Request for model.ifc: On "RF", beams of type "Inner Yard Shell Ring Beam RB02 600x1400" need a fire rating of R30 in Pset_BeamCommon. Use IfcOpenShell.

First a look at what the model holds.

```python
import ifcopenshell
import ifcopenshell.util.element

model = ifcopenshell.open("model.ifc")
print(model.schema)
storey = next(s for s in model.by_type("IfcBuildingStorey") if s.Name == "RF")
beams = [e for e in ifcopenshell.util.element.get_decomposition(storey) if e.is_a("IfcBeam")]
seen = {}
for e in beams:
    element_type = ifcopenshell.util.element.get_type(e)
    key = (element_type.Name if element_type != e and element_type else None, ifcopenshell.util.element.get_pset(e, "Pset_BeamCommon", "FireRating"))
    seen[key] = seen.get(key, 0) + 1
for (name, value), count in sorted(seen.items(), key=str):
    print(count, "x", name, "|", value)
```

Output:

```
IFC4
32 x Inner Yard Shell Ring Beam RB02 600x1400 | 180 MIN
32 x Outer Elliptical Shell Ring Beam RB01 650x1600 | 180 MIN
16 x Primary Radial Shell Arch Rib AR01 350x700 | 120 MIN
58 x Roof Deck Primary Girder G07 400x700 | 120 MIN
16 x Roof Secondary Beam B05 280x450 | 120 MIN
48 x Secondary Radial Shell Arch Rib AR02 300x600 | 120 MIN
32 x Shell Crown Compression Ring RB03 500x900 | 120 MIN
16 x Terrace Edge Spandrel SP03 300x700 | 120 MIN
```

```python
import ifcopenshell
import ifcopenshell.api.pset
import ifcopenshell.util.element

model = ifcopenshell.open("model.ifc")

storey = next(s for s in model.by_type("IfcBuildingStorey") if s.Name == "RF")
beams = [e for e in ifcopenshell.util.element.get_decomposition(storey) if e.is_a("IfcBeam")]

count = 0
for e in beams:
    element_type = ifcopenshell.util.element.get_type(e)
    if element_type in (None, e) or element_type.Name != "Inner Yard Shell Ring Beam RB02 600x1400":
        continue
    # add_pset returns the element's existing set when there is one.
    pset = ifcopenshell.api.pset.add_pset(model, product=e, name="Pset_BeamCommon")
    ifcopenshell.api.pset.edit_pset(model, pset=pset, properties={"FireRating": "R30"})
    count += 1

print(count, "beams updated")

model.write("model_edited.ifc")
```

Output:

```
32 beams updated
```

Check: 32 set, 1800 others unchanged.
